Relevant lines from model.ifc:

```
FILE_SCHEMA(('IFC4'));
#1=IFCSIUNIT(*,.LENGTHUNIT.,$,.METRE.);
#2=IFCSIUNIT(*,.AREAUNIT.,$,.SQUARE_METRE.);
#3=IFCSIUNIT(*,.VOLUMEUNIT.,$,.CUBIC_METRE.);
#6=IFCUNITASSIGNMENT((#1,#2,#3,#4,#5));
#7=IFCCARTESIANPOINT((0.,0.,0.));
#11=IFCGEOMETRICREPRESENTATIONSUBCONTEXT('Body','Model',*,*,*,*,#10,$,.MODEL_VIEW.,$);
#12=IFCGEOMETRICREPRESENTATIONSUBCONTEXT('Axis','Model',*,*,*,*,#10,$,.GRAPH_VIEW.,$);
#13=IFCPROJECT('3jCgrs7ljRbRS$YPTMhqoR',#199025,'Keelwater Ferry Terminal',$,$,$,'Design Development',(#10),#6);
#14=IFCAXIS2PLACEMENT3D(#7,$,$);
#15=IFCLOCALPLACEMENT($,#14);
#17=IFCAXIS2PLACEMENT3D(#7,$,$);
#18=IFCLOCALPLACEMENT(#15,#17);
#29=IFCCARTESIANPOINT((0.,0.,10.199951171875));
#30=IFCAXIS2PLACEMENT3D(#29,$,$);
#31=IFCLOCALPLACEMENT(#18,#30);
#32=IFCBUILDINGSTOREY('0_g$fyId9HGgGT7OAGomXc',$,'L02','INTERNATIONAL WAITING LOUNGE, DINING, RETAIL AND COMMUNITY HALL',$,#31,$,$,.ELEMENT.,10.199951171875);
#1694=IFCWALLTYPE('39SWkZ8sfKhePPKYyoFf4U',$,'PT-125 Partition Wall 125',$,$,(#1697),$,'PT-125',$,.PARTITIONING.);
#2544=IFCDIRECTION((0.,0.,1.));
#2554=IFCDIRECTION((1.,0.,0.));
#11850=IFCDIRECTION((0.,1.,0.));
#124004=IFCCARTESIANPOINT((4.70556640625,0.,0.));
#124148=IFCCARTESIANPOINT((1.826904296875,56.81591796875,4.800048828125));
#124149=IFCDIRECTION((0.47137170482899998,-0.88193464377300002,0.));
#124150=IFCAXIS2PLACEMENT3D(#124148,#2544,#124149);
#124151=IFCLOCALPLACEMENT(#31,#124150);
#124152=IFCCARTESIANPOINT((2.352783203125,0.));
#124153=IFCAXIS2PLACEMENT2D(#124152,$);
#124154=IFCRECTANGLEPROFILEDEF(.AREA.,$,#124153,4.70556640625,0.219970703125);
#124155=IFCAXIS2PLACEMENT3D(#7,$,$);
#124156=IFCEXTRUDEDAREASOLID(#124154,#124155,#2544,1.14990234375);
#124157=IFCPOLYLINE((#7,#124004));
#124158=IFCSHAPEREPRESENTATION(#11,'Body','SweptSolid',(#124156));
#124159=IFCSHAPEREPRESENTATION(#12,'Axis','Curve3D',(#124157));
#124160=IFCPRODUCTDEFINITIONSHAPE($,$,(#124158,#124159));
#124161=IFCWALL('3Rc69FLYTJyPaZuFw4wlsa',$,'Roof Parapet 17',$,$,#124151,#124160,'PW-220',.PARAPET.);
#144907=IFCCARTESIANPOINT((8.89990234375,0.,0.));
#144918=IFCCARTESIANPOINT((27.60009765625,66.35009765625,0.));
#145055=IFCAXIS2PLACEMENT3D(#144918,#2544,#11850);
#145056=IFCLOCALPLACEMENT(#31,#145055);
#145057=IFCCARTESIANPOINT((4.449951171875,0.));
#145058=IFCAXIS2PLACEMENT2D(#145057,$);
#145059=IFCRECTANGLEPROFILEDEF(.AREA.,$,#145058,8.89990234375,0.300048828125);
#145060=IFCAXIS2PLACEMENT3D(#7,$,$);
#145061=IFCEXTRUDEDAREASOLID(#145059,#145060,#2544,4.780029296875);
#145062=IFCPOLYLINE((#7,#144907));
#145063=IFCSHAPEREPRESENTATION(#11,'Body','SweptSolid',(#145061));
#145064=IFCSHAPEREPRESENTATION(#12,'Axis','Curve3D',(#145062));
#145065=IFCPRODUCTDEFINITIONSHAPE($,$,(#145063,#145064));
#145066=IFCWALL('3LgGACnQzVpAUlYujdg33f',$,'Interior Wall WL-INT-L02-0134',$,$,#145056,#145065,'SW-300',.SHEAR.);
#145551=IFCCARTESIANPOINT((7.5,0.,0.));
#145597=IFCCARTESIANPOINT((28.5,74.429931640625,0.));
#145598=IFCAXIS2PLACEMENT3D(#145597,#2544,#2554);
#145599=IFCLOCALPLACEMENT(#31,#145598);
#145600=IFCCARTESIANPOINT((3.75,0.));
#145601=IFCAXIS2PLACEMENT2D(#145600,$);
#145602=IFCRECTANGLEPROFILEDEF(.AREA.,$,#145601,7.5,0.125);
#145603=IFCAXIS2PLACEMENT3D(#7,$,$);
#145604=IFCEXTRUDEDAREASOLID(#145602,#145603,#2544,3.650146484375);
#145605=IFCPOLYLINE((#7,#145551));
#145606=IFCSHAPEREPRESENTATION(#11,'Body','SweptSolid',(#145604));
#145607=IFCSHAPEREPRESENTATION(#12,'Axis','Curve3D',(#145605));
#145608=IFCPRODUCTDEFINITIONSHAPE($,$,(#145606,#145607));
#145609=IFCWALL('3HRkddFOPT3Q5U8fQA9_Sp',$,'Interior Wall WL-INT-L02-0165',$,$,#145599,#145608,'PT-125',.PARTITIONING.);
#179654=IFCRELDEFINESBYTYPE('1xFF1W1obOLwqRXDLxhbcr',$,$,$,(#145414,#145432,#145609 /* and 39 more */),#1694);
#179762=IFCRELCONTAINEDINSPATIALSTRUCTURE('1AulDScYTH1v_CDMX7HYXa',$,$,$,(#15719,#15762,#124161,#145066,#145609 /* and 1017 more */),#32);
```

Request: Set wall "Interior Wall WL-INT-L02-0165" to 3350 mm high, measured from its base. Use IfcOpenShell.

```python
import ifcopenshell
import ifcopenshell.geom
import ifcopenshell.util.representation
import ifcopenshell.util.shape

model = ifcopenshell.open("model.ifc")
settings = ifcopenshell.geom.settings()


def volume(element):
    """Net volume in cubic metres, openings subtracted."""
    shape = ifcopenshell.geom.create_shape(settings, element)
    return ifcopenshell.util.shape.get_volume(shape.geometry)


wall = model.by_guid("3HRkddFOPT3Q5U8fQA9_Sp")
before = volume(wall)

body = ifcopenshell.util.representation.get_representation(wall, "Model", "Body")
solid = body.Items[0]
old_height = solid.Depth
solid.Depth = 3.35
after = volume(wall)

print(f"height {old_height:g} -> {solid.Depth:g}, volume {before:.3f} -> {after:.3f} m3")

model.write("model_updated.ifc")
```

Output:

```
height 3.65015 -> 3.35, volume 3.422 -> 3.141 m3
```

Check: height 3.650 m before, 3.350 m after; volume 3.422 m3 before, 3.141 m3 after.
